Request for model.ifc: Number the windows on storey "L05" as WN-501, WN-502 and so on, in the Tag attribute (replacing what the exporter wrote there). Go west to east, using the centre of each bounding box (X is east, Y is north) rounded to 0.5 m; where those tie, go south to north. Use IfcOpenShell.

First a look at what the model holds.

```python
import ifcopenshell
import ifcopenshell.util.element
import ifcopenshell.util.placement

model = ifcopenshell.open("model.ifc")
print(model.schema)
storey = next(s for s in model.by_type("IfcBuildingStorey") if s.Name == "L05")
windows = [e for e in ifcopenshell.util.element.get_decomposition(storey) if e.is_a("IfcWindow")]
for e in sorted(windows, key=lambda e: e.id()):
    origin = ifcopenshell.util.placement.get_local_placement(e.ObjectPlacement)[:3, 3]
    print(e.id(), e.Tag, e.Name, origin.round(2) + 0.0, sep=" | ")
```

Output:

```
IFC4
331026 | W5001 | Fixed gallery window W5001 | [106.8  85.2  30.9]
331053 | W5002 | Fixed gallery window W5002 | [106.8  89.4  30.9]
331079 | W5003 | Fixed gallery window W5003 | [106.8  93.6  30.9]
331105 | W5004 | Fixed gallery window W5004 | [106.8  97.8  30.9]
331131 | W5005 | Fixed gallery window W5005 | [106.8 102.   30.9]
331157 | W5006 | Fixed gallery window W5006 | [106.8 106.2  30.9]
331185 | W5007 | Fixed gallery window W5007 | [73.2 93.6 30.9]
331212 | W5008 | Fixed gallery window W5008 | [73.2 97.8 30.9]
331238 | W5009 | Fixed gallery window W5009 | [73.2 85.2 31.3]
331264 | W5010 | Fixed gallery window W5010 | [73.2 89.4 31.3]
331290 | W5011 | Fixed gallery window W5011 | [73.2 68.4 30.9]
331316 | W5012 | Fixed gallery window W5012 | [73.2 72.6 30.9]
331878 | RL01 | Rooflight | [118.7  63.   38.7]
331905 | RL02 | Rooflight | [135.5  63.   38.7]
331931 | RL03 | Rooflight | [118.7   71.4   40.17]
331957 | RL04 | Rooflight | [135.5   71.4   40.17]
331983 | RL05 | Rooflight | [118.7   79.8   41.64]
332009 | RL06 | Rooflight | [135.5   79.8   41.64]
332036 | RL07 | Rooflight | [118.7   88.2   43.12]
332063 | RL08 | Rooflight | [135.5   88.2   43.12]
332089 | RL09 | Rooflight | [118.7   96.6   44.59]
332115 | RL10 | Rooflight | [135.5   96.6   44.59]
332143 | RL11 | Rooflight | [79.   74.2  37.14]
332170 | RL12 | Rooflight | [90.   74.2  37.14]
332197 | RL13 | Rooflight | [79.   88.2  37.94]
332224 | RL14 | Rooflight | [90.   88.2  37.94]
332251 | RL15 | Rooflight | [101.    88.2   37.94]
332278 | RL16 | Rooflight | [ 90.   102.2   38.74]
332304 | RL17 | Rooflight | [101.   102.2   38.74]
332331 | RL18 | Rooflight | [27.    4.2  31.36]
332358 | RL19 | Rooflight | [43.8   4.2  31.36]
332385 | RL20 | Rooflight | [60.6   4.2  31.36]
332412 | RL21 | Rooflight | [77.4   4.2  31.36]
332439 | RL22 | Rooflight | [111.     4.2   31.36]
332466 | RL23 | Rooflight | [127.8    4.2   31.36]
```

```python
import ifcopenshell
import ifcopenshell.geom
import ifcopenshell.util.element
import ifcopenshell.util.shape

model = ifcopenshell.open("model.ifc")
settings = ifcopenshell.geom.settings()
settings.set("use-world-coords", True)


def centre(element):
    shape = ifcopenshell.geom.create_shape(settings, element)
    return ifcopenshell.util.shape.get_bbox_centroid(shape.geometry)


storey = next(s for s in model.by_type("IfcBuildingStorey") if s.Name == "L05")
windows = [e for e in ifcopenshell.util.element.get_decomposition(storey) if e.is_a("IfcWindow")]

# Insertion points can sit at a corner or the storey origin, so sort by the geometry (in metres).
centres = {e: centre(e) for e in windows}
windows.sort(key=lambda e: (round(centres[e][0] / 0.5), centres[e][1]))

for i, e in enumerate(windows, start=1):
    number = f"WN-5{i:02d}"
    e.Tag = number
    print(e.id(), number)

model.write("model_v2.ifc")
```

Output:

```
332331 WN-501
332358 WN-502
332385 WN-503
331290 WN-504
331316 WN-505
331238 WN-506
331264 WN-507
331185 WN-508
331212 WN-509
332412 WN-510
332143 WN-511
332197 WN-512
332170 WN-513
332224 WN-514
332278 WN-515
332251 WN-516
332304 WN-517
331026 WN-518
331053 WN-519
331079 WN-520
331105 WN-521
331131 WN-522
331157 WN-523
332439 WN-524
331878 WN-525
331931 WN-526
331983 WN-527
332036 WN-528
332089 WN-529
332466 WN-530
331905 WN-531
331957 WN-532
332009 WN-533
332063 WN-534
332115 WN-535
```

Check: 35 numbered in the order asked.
